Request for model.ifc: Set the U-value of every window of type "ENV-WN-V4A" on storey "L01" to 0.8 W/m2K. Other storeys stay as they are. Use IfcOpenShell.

First a look at what the model holds.

```python
import ifcopenshell
import ifcopenshell.util.element

model = ifcopenshell.open("model.ifc")
print(model.schema)
storey = next(s for s in model.by_type("IfcBuildingStorey") if s.Name == "L01")
windows = [e for e in ifcopenshell.util.element.get_decomposition(storey) if e.is_a("IfcWindow")]
seen = {}
for e in windows:
    element_type = ifcopenshell.util.element.get_type(e)
    key = (element_type.Name if element_type != e and element_type else None, ifcopenshell.util.element.get_pset(e, "Pset_WindowCommon", "ThermalTransmittance"))
    seen[key] = seen.get(key, 0) + 1
for (name, value), count in sorted(seen.items(), key=str):
    print(count, "x", name, "|", value)
```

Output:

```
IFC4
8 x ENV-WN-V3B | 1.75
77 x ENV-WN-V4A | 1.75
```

```python
import ifcopenshell
import ifcopenshell.api.pset
import ifcopenshell.util.element

model = ifcopenshell.open("model.ifc")

storey = next(s for s in model.by_type("IfcBuildingStorey") if s.Name == "L01")
windows = [e for e in ifcopenshell.util.element.get_decomposition(storey) if e.is_a("IfcWindow")]

count = 0
for e in windows:
    element_type = ifcopenshell.util.element.get_type(e)
    if element_type in (None, e) or element_type.Name != "ENV-WN-V4A":
        continue
    # add_pset returns the element's existing set when there is one.
    pset = ifcopenshell.api.pset.add_pset(model, product=e, name="Pset_WindowCommon")
    ifcopenshell.api.pset.edit_pset(model, pset=pset, properties={"ThermalTransmittance": 0.8})
    count += 1

print(count, "windows updated")

model.write("model_rev.ifc")
```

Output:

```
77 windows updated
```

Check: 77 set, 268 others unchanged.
